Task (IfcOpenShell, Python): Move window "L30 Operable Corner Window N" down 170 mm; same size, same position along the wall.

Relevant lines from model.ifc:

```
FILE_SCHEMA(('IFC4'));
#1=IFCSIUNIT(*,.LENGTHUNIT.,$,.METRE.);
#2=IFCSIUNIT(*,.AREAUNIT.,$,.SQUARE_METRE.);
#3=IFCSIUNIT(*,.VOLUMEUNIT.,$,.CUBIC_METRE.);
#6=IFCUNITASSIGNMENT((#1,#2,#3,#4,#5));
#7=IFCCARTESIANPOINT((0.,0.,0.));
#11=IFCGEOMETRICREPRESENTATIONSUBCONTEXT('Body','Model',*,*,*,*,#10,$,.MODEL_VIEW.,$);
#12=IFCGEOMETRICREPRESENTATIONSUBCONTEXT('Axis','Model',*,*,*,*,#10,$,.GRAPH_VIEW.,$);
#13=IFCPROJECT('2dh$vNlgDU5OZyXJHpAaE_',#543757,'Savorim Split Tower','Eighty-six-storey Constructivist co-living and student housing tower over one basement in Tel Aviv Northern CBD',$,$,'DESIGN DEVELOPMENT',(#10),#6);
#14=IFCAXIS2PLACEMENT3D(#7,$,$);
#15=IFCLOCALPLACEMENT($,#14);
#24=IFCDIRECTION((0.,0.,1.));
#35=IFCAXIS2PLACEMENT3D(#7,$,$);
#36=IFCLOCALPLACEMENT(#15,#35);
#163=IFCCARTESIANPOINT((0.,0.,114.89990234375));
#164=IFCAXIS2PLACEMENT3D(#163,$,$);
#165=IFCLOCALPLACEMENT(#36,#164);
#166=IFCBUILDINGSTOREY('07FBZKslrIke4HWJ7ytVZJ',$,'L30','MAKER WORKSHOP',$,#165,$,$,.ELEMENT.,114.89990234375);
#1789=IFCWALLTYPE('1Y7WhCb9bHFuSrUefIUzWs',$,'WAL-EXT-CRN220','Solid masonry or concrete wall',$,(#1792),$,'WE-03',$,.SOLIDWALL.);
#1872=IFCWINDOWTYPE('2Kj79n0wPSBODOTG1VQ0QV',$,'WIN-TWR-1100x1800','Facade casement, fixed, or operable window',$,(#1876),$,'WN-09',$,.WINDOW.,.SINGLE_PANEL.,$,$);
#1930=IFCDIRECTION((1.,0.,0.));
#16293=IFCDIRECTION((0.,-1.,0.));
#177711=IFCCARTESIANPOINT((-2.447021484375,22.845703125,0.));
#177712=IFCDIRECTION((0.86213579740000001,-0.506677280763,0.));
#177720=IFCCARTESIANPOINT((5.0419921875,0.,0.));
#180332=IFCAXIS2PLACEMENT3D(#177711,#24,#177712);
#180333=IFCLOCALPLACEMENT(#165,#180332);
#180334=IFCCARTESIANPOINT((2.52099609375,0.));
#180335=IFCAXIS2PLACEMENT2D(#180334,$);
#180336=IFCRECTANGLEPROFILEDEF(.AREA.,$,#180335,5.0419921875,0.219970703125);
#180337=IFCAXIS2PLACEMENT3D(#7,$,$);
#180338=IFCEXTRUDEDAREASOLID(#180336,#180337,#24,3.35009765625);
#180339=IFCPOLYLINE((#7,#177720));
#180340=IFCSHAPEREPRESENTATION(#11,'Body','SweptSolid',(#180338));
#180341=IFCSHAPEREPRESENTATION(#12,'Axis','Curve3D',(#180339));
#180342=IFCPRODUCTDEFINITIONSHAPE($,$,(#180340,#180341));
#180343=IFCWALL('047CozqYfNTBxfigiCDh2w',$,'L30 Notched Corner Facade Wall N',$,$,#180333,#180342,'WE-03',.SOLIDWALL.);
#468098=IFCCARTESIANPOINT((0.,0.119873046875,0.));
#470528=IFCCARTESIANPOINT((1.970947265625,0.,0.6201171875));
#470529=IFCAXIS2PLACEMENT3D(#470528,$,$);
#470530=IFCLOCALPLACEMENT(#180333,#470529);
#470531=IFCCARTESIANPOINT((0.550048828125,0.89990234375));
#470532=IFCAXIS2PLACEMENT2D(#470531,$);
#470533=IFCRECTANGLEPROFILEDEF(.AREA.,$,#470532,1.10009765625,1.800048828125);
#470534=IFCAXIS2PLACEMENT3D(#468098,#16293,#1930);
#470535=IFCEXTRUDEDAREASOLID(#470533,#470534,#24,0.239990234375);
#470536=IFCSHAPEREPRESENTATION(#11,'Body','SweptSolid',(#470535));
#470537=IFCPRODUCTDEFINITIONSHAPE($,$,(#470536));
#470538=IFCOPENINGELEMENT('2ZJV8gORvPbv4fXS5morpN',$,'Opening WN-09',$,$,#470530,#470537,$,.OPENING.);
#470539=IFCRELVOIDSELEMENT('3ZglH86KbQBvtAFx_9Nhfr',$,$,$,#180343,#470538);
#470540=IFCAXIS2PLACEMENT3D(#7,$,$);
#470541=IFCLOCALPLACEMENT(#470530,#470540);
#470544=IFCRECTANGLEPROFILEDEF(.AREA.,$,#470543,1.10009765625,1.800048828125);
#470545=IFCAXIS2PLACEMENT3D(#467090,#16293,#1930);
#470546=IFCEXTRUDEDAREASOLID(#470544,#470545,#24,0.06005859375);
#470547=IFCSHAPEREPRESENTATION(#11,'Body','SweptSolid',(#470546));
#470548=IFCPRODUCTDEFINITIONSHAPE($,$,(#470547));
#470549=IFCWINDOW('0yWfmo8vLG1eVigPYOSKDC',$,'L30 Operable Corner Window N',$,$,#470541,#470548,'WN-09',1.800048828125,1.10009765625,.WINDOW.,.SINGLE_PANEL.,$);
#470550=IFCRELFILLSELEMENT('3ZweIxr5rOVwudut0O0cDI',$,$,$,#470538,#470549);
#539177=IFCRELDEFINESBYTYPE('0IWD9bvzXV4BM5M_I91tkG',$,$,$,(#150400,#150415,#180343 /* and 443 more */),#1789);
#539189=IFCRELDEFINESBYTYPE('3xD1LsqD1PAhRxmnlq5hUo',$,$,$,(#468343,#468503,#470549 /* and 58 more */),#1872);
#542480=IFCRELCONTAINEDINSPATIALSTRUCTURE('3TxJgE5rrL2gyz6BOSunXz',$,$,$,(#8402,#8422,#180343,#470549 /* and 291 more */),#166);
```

```python
import numpy as np
import ifcopenshell
import ifcopenshell.api.geometry
import ifcopenshell.util.placement
import ifcopenshell.util.unit

model = ifcopenshell.open("model.ifc")
unit_scale = ifcopenshell.util.unit.calculate_unit_scale(model)

window = model.by_id(470549)
opening = window.FillsVoids[0].RelatingOpeningElement
dz = -0.17 / unit_scale

shift = np.array([0.0, 0.0, dz])
# The window is placed relative to its opening, so it follows when the opening moves.
matrix = ifcopenshell.util.placement.get_local_placement(opening.ObjectPlacement)
matrix[:3, 3] += shift
ifcopenshell.api.geometry.edit_object_placement(
    model, product=opening, matrix=matrix, is_si=False, should_transform_children=True
)

print(f"moved by {dz * unit_scale:+.3f} m")

model.write("model_rev.ifc")
```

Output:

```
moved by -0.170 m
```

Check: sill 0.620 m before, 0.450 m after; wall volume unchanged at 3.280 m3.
